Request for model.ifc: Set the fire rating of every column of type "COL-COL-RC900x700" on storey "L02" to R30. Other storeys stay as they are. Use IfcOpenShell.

First a look at what the model holds.

```python
import ifcopenshell
import ifcopenshell.util.element

model = ifcopenshell.open("model.ifc")
print(model.schema)
storey = next(s for s in model.by_type("IfcBuildingStorey") if s.Name == "L02")
columns = [e for e in ifcopenshell.util.element.get_decomposition(storey) if e.is_a("IfcColumn")]
seen = {}
for e in columns:
    element_type = ifcopenshell.util.element.get_type(e)
    key = (element_type.Name if element_type != e and element_type else None, ifcopenshell.util.element.get_pset(e, "Pset_ColumnCommon", "FireRating"))
    seen[key] = seen.get(key, 0) + 1
for (name, value), count in sorted(seen.items(), key=str):
    print(count, "x", name, "|", value)
```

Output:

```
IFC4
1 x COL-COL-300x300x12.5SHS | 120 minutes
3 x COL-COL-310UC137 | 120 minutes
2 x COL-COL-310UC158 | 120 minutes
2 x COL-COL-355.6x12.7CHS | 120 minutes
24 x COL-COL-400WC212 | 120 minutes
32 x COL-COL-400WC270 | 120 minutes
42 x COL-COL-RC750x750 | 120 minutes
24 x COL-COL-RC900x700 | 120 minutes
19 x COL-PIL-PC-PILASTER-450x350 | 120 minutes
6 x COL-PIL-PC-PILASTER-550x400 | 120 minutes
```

```python
import ifcopenshell
import ifcopenshell.api.pset
import ifcopenshell.util.element

model = ifcopenshell.open("model.ifc")

storey = next(s for s in model.by_type("IfcBuildingStorey") if s.Name == "L02")
columns = [e for e in ifcopenshell.util.element.get_decomposition(storey) if e.is_a("IfcColumn")]

count = 0
for e in columns:
    element_type = ifcopenshell.util.element.get_type(e)
    if element_type in (None, e) or element_type.Name != "COL-COL-RC900x700":
        continue
    # add_pset returns the element's existing set when there is one.
    pset = ifcopenshell.api.pset.add_pset(model, product=e, name="Pset_ColumnCommon")
    ifcopenshell.api.pset.edit_pset(model, pset=pset, properties={"FireRating": "R30"})
    count += 1

print(count, "columns updated")

model.write("model-out.ifc")
```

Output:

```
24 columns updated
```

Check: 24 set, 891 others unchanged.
